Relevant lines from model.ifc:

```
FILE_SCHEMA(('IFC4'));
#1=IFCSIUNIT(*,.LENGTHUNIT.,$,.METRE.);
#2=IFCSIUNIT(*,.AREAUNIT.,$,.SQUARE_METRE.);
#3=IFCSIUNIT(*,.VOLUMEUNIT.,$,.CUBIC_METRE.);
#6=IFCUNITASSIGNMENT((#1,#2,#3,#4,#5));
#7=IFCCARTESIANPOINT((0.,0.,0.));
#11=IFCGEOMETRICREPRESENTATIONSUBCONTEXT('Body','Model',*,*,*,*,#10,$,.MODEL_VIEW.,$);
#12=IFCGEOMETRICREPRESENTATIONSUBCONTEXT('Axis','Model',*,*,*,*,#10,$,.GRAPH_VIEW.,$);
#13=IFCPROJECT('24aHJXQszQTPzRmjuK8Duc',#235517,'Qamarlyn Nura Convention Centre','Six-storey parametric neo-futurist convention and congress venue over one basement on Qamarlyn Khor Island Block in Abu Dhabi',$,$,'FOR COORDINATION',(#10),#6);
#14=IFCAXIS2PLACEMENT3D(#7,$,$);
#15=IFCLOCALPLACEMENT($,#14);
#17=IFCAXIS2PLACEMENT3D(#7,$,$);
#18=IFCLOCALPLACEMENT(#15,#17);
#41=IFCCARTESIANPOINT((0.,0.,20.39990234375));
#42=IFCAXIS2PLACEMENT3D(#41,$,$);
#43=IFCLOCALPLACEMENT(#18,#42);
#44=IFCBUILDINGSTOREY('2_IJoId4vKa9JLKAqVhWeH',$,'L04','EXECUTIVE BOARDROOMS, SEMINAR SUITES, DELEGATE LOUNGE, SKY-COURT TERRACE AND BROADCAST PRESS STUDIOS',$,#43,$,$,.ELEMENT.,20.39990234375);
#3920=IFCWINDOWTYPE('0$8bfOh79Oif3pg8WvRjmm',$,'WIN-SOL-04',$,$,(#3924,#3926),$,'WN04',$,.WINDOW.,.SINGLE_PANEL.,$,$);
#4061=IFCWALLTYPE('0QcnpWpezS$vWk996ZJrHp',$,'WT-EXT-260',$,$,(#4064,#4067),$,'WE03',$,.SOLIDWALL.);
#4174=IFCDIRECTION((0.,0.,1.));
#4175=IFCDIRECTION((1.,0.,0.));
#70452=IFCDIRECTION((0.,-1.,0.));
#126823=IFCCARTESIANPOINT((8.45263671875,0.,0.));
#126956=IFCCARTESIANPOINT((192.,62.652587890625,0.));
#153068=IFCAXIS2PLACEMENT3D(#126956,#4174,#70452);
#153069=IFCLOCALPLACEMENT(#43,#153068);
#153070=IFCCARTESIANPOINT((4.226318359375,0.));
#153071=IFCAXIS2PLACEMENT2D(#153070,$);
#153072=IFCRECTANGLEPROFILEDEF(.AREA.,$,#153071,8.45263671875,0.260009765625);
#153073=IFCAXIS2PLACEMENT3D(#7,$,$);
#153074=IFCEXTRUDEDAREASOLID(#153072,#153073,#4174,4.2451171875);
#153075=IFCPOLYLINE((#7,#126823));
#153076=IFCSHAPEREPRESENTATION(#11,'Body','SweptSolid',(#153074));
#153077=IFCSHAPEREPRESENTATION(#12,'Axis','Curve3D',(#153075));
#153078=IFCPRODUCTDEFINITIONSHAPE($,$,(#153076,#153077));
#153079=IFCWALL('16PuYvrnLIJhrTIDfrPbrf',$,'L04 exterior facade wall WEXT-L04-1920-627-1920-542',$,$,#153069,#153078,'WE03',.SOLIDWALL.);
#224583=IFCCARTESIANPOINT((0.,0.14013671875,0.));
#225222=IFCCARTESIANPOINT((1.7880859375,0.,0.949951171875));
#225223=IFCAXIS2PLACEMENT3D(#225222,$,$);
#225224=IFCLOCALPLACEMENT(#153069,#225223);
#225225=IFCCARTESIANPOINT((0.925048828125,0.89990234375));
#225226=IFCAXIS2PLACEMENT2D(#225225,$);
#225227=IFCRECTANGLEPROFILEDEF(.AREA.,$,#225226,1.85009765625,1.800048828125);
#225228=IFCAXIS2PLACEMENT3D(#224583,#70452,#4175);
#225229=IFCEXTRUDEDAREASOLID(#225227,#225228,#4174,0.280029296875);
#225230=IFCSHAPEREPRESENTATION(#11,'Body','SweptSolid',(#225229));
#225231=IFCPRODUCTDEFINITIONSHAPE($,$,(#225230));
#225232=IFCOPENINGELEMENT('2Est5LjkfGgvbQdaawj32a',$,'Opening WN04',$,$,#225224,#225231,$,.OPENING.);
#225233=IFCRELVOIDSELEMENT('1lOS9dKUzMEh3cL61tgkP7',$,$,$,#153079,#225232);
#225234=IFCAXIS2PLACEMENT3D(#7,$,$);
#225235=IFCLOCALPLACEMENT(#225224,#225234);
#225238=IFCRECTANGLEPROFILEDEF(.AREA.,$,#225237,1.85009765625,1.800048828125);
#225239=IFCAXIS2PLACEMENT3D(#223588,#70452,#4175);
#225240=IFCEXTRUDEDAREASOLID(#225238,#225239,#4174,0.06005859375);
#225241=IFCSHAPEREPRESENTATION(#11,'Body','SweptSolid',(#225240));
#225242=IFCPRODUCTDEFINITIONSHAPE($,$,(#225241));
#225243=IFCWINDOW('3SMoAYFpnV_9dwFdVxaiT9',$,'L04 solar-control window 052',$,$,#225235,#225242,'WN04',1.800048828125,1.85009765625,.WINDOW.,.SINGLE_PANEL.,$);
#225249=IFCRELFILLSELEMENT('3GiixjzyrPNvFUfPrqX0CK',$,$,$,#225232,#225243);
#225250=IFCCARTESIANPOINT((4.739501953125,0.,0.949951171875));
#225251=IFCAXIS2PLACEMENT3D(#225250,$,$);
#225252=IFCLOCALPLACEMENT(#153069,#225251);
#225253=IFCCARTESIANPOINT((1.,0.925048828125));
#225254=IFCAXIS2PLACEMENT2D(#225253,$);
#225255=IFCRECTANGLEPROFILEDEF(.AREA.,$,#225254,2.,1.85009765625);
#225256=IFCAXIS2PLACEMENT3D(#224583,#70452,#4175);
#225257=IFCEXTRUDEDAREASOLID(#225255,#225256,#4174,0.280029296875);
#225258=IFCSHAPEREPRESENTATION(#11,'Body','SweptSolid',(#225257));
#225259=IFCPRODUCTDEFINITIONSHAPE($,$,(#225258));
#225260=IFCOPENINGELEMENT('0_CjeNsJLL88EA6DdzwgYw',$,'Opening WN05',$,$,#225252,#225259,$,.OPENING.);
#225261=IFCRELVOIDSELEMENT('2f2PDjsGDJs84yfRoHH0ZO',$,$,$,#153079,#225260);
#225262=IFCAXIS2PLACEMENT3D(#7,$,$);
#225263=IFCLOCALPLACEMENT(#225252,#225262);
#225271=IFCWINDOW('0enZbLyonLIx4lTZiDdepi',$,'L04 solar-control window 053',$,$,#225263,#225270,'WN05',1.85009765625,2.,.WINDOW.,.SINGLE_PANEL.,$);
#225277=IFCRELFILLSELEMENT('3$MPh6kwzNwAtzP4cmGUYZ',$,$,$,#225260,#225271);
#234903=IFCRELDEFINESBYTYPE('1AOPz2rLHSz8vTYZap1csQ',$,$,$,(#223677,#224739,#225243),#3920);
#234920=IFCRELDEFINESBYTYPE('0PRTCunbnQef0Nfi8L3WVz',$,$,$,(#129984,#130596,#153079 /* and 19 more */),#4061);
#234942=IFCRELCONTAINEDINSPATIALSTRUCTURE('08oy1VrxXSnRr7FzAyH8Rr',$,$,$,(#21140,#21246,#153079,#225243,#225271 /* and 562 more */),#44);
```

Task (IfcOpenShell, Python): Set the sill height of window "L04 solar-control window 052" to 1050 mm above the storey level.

```python
import numpy as np
import ifcopenshell
import ifcopenshell.api.geometry
import ifcopenshell.geom
import ifcopenshell.util.element
import ifcopenshell.util.placement
import ifcopenshell.util.shape
import ifcopenshell.util.unit

model = ifcopenshell.open("model.ifc")
unit_scale = ifcopenshell.util.unit.calculate_unit_scale(model)

window = model.by_guid("3SMoAYFpnV_9dwFdVxaiT9")
opening = window.FillsVoids[0].RelatingOpeningElement
storey = ifcopenshell.util.element.get_container(window, ifc_class="IfcBuildingStorey")
level = ifcopenshell.util.placement.get_local_placement(storey.ObjectPlacement)[2, 3]

# The opening's origin need not be at the sill, so measure its lowest point.
shape = ifcopenshell.geom.create_shape(ifcopenshell.geom.settings(), opening)
bottom = ifcopenshell.util.shape.get_shape_bottom_elevation(shape, shape.geometry) / unit_scale
dz = level + 1.05 / unit_scale - bottom

shift = np.array([0.0, 0.0, dz])
# The window is placed relative to its opening, so it follows when the opening moves.
matrix = ifcopenshell.util.placement.get_local_placement(opening.ObjectPlacement)
matrix[:3, 3] += shift
ifcopenshell.api.geometry.edit_object_placement(
    model, product=opening, matrix=matrix, is_si=False, should_transform_children=True
)

print(f"moved by {dz * unit_scale:+.3f} m")

model.write("model-out.ifc")
```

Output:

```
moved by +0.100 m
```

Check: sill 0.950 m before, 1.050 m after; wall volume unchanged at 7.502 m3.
